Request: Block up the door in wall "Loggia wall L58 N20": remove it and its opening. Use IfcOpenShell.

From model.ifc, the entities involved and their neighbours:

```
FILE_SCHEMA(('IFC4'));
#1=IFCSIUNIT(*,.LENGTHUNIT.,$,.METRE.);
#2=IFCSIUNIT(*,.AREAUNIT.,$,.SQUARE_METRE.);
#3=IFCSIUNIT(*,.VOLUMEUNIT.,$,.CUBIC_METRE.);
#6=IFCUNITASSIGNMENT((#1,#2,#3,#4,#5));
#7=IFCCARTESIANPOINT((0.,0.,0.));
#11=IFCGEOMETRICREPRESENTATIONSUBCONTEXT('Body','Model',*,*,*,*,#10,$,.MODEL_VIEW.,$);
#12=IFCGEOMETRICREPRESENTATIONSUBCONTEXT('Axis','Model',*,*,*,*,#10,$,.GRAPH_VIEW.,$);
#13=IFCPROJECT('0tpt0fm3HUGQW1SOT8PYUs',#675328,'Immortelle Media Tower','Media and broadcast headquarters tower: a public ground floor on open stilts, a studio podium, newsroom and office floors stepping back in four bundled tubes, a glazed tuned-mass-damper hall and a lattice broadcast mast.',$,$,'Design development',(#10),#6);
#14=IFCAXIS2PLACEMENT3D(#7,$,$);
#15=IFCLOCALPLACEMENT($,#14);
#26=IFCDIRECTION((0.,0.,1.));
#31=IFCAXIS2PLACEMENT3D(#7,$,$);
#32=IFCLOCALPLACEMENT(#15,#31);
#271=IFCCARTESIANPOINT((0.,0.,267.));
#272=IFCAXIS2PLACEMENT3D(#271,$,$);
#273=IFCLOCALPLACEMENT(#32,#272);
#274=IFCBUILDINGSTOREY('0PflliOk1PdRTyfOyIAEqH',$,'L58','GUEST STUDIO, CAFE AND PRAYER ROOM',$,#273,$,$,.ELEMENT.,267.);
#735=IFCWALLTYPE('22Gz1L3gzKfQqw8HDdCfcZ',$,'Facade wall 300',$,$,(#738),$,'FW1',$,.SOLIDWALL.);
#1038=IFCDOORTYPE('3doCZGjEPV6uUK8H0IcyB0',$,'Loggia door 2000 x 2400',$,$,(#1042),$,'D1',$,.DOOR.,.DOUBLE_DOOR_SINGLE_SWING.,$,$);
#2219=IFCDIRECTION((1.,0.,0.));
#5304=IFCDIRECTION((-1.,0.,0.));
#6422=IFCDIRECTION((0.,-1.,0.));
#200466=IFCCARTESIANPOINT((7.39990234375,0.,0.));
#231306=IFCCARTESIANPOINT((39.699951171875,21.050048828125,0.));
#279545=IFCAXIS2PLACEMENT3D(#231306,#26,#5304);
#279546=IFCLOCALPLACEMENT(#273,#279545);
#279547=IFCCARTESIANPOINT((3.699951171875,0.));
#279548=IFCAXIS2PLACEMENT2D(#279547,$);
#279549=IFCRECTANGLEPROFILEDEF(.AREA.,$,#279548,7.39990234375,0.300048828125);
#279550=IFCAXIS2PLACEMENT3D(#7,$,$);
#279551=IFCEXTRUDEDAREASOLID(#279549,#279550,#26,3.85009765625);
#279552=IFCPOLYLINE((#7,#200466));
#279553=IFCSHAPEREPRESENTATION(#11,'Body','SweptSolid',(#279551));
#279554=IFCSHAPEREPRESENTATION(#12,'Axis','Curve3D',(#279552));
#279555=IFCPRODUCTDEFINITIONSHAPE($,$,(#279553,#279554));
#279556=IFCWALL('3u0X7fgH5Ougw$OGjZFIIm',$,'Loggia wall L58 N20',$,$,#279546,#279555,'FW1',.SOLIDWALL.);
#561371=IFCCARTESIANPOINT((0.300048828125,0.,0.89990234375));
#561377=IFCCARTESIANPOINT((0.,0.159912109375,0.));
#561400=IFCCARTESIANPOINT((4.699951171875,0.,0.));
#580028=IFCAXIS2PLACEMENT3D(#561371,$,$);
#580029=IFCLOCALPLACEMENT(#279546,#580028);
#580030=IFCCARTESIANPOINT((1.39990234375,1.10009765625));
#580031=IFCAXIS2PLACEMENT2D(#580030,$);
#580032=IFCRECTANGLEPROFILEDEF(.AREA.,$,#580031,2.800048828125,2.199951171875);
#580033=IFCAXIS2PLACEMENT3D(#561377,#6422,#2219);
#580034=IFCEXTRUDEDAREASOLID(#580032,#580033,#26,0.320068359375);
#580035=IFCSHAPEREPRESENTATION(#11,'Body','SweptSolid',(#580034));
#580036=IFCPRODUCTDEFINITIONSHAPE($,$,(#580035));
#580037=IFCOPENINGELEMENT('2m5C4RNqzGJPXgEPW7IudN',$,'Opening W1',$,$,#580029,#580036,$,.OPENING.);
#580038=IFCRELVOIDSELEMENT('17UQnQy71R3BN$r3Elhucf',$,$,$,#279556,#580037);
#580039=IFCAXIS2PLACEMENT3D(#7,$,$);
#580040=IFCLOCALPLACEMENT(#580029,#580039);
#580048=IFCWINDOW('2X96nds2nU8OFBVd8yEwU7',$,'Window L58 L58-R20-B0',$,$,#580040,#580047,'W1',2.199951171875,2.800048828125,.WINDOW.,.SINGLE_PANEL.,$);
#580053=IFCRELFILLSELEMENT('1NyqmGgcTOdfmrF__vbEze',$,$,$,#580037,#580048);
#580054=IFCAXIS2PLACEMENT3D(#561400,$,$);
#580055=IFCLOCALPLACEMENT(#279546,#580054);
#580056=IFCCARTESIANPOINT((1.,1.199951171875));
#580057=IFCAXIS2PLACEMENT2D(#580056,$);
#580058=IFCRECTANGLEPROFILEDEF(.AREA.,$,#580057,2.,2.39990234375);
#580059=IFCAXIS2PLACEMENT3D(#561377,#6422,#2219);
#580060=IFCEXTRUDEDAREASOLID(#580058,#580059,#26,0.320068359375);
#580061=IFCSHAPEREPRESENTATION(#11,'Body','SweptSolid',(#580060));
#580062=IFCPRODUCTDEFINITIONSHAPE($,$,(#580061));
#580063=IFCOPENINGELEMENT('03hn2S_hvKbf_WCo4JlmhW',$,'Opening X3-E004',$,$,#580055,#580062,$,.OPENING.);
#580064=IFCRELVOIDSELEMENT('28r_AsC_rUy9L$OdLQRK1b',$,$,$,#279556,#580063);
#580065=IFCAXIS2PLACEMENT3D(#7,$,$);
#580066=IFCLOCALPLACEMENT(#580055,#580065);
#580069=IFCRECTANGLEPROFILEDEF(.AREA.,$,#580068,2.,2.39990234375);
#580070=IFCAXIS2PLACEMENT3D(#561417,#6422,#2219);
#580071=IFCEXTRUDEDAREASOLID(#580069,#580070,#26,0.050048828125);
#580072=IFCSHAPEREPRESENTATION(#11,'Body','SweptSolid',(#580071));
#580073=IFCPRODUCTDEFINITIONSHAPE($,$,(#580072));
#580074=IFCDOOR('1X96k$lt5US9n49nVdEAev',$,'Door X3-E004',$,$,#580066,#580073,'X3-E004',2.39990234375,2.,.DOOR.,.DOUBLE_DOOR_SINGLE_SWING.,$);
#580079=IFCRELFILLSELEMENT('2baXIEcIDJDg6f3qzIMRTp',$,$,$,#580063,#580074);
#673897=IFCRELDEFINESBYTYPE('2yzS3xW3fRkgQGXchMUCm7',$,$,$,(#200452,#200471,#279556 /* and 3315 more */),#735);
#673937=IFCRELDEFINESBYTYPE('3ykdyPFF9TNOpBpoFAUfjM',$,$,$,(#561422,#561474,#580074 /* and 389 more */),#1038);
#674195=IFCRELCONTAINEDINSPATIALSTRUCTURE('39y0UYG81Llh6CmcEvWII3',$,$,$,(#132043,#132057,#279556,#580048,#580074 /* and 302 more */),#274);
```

```python
import ifcopenshell
import ifcopenshell.api.feature
import ifcopenshell.api.root
import ifcopenshell.geom
import ifcopenshell.util.shape

model = ifcopenshell.open("model.ifc")
settings = ifcopenshell.geom.settings()


def volume(element):
    """Net volume in cubic metres, openings subtracted."""
    shape = ifcopenshell.geom.create_shape(settings, element)
    return ifcopenshell.util.shape.get_volume(shape.geometry)


door = model.by_guid("1X96k$lt5US9n49nVdEAev")
opening = door.FillsVoids[0].RelatingOpeningElement
wall = opening.VoidsElements[0].RelatingBuildingElement
before = volume(wall)

ifcopenshell.api.root.remove_product(model, product=door)
ifcopenshell.api.feature.remove_feature(model, feature=opening)

after = volume(wall)

print(f"wall volume {before:.3f} -> {after:.3f} m3")

model.write("model_updated.ifc")
```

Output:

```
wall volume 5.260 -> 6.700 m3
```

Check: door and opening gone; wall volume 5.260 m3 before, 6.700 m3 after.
